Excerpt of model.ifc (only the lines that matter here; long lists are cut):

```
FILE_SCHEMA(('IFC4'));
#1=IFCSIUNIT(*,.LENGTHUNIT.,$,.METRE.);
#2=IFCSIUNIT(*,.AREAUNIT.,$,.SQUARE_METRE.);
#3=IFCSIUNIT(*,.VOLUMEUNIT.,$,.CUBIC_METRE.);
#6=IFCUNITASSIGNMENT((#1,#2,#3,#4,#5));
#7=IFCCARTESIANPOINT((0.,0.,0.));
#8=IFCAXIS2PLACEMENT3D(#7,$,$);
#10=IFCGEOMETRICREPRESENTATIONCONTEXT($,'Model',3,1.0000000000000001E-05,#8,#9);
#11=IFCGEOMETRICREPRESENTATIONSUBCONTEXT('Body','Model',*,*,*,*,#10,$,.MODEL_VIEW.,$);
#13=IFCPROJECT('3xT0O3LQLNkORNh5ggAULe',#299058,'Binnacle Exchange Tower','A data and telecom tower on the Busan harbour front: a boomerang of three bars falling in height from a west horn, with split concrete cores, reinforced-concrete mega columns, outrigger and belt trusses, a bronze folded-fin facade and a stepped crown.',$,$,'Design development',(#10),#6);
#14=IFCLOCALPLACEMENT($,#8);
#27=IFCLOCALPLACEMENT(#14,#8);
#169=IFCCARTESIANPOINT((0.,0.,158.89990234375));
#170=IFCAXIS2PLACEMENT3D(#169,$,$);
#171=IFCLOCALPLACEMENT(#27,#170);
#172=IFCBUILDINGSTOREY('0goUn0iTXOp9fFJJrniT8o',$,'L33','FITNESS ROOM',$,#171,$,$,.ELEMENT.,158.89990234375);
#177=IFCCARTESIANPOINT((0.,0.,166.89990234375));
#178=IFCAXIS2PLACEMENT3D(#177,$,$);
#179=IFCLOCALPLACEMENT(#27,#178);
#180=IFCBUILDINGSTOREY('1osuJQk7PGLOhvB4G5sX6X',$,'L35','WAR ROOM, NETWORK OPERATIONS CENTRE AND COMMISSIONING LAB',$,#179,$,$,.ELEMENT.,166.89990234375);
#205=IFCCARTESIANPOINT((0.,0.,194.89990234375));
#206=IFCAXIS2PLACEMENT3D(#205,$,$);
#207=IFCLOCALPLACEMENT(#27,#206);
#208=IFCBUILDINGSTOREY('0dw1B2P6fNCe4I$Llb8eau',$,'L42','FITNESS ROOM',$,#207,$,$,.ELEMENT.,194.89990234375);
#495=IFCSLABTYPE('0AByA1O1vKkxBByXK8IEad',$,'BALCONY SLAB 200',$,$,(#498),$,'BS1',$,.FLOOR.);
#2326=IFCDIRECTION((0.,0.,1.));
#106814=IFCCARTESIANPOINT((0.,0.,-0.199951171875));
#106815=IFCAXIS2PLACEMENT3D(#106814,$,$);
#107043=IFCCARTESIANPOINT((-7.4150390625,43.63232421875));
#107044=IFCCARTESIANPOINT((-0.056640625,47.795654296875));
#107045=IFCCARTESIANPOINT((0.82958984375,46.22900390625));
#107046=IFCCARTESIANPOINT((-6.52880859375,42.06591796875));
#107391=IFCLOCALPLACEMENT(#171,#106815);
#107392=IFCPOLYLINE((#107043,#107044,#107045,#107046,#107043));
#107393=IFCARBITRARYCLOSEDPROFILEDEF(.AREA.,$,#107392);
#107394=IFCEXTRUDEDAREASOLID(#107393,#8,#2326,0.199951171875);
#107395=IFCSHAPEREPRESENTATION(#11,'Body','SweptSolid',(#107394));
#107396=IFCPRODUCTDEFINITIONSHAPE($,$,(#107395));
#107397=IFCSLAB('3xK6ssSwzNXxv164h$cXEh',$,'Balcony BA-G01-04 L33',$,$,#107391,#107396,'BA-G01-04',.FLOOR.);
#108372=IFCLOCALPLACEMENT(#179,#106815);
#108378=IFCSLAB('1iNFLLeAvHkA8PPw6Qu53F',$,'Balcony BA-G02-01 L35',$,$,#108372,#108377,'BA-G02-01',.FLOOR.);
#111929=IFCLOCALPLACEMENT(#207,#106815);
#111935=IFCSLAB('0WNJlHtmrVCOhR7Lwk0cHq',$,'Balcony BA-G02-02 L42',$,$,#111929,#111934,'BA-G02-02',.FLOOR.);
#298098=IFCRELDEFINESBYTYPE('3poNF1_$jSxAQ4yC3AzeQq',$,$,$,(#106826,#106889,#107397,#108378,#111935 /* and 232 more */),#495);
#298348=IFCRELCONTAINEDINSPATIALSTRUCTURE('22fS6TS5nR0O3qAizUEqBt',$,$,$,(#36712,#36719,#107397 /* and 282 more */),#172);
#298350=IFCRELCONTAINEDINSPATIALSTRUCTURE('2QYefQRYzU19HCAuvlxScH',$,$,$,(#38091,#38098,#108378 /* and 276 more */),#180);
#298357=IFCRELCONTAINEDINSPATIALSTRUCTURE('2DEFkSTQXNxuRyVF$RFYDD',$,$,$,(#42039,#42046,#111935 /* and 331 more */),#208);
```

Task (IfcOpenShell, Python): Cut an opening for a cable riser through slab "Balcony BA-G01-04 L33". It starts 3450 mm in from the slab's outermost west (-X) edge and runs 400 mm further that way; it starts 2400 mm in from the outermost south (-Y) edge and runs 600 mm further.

```python
import numpy as np
import ifcopenshell
import ifcopenshell.api.feature
import ifcopenshell.api.geometry
import ifcopenshell.api.root
import ifcopenshell.geom
import ifcopenshell.util.placement
import ifcopenshell.util.representation
import ifcopenshell.util.shape
import ifcopenshell.util.unit

model = ifcopenshell.open("model.ifc")
unit_scale = ifcopenshell.util.unit.calculate_unit_scale(model)
settings = ifcopenshell.geom.settings()


def volume(element):
    """Net volume in cubic metres, openings subtracted."""
    shape = ifcopenshell.geom.create_shape(settings, element)
    return ifcopenshell.util.shape.get_volume(shape.geometry)


slab = model.by_guid("3xK6ssSwzNXxv164h$cXEh")
before = volume(slab)

# Extent in the slab's own axes, in metres. The edges named are its -X and -Y sides.
slab_shape = ifcopenshell.geom.create_shape(settings, slab)
vertices = ifcopenshell.util.shape.get_vertices(slab_shape.geometry)
x_min, y_min, bottom = vertices.min(axis=0)
top = vertices[:, 2].max()

opening = ifcopenshell.api.root.create_entity(model, ifc_class="IfcOpeningElement", name="Cable riser opening", predefined_type="OPENING")
context = ifcopenshell.util.representation.get_context(model, "Model", "Body", "MODEL_VIEW")
width, depth = 0.4, 0.6
outline = [(0.0, 0.0), (width, 0.0), (width, depth), (0.0, depth), (0.0, 0.0)]
# Overshoot both faces by 50 mm so the cut is clean.
shape = ifcopenshell.api.geometry.add_slab_representation(
    model, context=context, depth=top - bottom + 0.1, polyline=outline
)
ifcopenshell.api.geometry.assign_representation(model, product=opening, representation=shape)

matrix = ifcopenshell.util.placement.get_local_placement(slab.ObjectPlacement)
matrix[:, 3] = matrix @ np.append(np.array([x_min + 3.45, y_min + 2.4, bottom - 0.05]) / unit_scale, 1.0)
ifcopenshell.api.geometry.edit_object_placement(model, product=opening, matrix=matrix, is_si=False)
ifcopenshell.api.feature.add_feature(model, feature=opening, element=slab)

after = volume(slab)

print(f"slab volume {before:.3f} -> {after:.3f} m3")

model.write("model_edited.ifc")
```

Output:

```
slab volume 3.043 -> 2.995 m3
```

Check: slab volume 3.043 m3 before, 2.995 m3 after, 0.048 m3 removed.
